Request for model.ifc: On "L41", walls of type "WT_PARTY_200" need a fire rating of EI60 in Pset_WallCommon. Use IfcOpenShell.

First a look at what the model holds.

```python
import ifcopenshell
import ifcopenshell.util.element

model = ifcopenshell.open("model.ifc")
print(model.schema)
storey = next(s for s in model.by_type("IfcBuildingStorey") if s.Name == "L41")
walls = [e for e in ifcopenshell.util.element.get_decomposition(storey) if e.is_a("IfcWall")]
seen = {}
for e in walls:
    element_type = ifcopenshell.util.element.get_type(e)
    key = (element_type.Name if element_type != e and element_type else None, ifcopenshell.util.element.get_pset(e, "Pset_WallCommon", "FireRating"))
    seen[key] = seen.get(key, 0) + 1
for (name, value), count in sorted(seen.items(), key=str):
    print(count, "x", name, "|", value)
```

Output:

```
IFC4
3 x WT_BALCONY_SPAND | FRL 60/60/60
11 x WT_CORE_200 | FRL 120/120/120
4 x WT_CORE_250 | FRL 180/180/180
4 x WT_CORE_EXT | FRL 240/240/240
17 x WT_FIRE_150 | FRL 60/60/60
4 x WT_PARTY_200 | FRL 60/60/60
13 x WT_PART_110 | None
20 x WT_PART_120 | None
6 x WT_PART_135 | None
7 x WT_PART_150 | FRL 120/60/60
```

```python
import ifcopenshell
import ifcopenshell.api.pset
import ifcopenshell.util.element

model = ifcopenshell.open("model.ifc")

storey = next(s for s in model.by_type("IfcBuildingStorey") if s.Name == "L41")
walls = [e for e in ifcopenshell.util.element.get_decomposition(storey) if e.is_a("IfcWall")]

count = 0
for e in walls:
    element_type = ifcopenshell.util.element.get_type(e)
    if element_type in (None, e) or element_type.Name != "WT_PARTY_200":
        continue
    # add_pset returns the element's existing set when there is one.
    pset = ifcopenshell.api.pset.add_pset(model, product=e, name="Pset_WallCommon")
    ifcopenshell.api.pset.edit_pset(model, pset=pset, properties={"FireRating": "EI60"})
    count += 1

print(count, "walls updated")

model.write("model_edited.ifc")
```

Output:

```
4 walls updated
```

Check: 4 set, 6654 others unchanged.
